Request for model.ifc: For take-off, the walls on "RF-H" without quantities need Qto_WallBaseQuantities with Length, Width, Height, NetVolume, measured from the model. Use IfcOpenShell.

First a look at what the model holds.

```python
import ifcopenshell
import ifcopenshell.util.element
import ifcopenshell.util.unit

model = ifcopenshell.open("model.ifc")
print(model.schema)
for unit_type in ("LENGTHUNIT", "AREAUNIT", "VOLUMEUNIT"):
    print(unit_type, ifcopenshell.util.unit.calculate_unit_scale(model, unit_type))
storey = next(s for s in model.by_type("IfcBuildingStorey") if s.Name == "RF-H")
walls = [e for e in ifcopenshell.util.element.get_decomposition(storey) if e.is_a("IfcWall")]
for e in sorted(walls, key=lambda e: e.id()):
    print(e.id(), e.is_a(), e.Name, list(ifcopenshell.util.element.get_psets(e, qtos_only=True)), sep=" | ")
```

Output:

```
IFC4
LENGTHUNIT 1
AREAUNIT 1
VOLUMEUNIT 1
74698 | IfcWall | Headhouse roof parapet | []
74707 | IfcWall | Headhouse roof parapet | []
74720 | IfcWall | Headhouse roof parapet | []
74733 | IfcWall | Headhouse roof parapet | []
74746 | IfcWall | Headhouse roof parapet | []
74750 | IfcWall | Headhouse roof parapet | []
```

```python
import ifcopenshell
import ifcopenshell.api.pset
import ifcopenshell.geom
import ifcopenshell.util.element
import ifcopenshell.util.shape
import ifcopenshell.util.unit

model = ifcopenshell.open("model.ifc")
unit_scale = ifcopenshell.util.unit.calculate_unit_scale(model)
volume_scale = ifcopenshell.util.unit.calculate_unit_scale(model, "VOLUMEUNIT")
settings = ifcopenshell.geom.settings()

storey = next(s for s in model.by_type("IfcBuildingStorey") if s.Name == "RF-H")
walls = [e for e in ifcopenshell.util.element.get_decomposition(storey) if e.is_a("IfcWall")]

for e in sorted(walls, key=lambda e: e.id()):
    if ifcopenshell.util.element.get_psets(e, qtos_only=True, should_inherit=False):
        continue
    # Geometry comes back in metres, in the element's own axes.
    shape = ifcopenshell.geom.create_shape(settings, e)
    values = {
        "Length": ifcopenshell.util.shape.get_x(shape.geometry) / unit_scale,
        "Width": ifcopenshell.util.shape.get_y(shape.geometry) / unit_scale,
        "Height": ifcopenshell.util.shape.get_z(shape.geometry) / unit_scale,
        "NetVolume": ifcopenshell.util.shape.get_volume(shape.geometry) / volume_scale,
    }
    qto = ifcopenshell.api.pset.add_qto(model, product=e, name="Qto_WallBaseQuantities")
    ifcopenshell.api.pset.edit_qto(model, qto=qto, properties=values)
    print(e.id(), {k: round(v, 3) for k, v in values.items()})

model.write("model_v2.ifc")
```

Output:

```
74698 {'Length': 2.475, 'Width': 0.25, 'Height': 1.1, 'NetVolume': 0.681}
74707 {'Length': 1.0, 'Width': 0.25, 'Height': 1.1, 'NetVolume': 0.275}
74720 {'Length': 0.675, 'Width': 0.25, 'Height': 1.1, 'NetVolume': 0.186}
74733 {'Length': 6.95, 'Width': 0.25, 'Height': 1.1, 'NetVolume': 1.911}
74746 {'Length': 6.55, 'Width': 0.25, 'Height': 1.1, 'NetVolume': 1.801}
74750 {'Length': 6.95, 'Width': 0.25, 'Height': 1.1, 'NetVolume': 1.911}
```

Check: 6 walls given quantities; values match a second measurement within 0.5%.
